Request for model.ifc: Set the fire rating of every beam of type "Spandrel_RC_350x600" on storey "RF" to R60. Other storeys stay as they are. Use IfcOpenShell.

First a look at what the model holds.

```python
import ifcopenshell
import ifcopenshell.util.element

model = ifcopenshell.open("model.ifc")
print(model.schema)
storey = next(s for s in model.by_type("IfcBuildingStorey") if s.Name == "RF")
beams = [e for e in ifcopenshell.util.element.get_decomposition(storey) if e.is_a("IfcBeam")]
seen = {}
for e in beams:
    element_type = ifcopenshell.util.element.get_type(e)
    key = (element_type.Name if element_type != e and element_type else None, ifcopenshell.util.element.get_pset(e, "Pset_BeamCommon", "FireRating"))
    seen[key] = seen.get(key, 0) + 1
for (name, value), count in sorted(seen.items(), key=str):
    print(count, "x", name, "|", value)
```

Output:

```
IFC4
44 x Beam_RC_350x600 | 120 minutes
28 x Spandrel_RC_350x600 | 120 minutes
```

```python
import ifcopenshell
import ifcopenshell.api.pset
import ifcopenshell.util.element

model = ifcopenshell.open("model.ifc")

storey = next(s for s in model.by_type("IfcBuildingStorey") if s.Name == "RF")
beams = [e for e in ifcopenshell.util.element.get_decomposition(storey) if e.is_a("IfcBeam")]

count = 0
for e in beams:
    element_type = ifcopenshell.util.element.get_type(e)
    if element_type in (None, e) or element_type.Name != "Spandrel_RC_350x600":
        continue
    # add_pset returns the element's existing set when there is one.
    pset = ifcopenshell.api.pset.add_pset(model, product=e, name="Pset_BeamCommon")
    ifcopenshell.api.pset.edit_pset(model, pset=pset, properties={"FireRating": "R60"})
    count += 1

print(count, "beams updated")

model.write("model_v2.ifc")
```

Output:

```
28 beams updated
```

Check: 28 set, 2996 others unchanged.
